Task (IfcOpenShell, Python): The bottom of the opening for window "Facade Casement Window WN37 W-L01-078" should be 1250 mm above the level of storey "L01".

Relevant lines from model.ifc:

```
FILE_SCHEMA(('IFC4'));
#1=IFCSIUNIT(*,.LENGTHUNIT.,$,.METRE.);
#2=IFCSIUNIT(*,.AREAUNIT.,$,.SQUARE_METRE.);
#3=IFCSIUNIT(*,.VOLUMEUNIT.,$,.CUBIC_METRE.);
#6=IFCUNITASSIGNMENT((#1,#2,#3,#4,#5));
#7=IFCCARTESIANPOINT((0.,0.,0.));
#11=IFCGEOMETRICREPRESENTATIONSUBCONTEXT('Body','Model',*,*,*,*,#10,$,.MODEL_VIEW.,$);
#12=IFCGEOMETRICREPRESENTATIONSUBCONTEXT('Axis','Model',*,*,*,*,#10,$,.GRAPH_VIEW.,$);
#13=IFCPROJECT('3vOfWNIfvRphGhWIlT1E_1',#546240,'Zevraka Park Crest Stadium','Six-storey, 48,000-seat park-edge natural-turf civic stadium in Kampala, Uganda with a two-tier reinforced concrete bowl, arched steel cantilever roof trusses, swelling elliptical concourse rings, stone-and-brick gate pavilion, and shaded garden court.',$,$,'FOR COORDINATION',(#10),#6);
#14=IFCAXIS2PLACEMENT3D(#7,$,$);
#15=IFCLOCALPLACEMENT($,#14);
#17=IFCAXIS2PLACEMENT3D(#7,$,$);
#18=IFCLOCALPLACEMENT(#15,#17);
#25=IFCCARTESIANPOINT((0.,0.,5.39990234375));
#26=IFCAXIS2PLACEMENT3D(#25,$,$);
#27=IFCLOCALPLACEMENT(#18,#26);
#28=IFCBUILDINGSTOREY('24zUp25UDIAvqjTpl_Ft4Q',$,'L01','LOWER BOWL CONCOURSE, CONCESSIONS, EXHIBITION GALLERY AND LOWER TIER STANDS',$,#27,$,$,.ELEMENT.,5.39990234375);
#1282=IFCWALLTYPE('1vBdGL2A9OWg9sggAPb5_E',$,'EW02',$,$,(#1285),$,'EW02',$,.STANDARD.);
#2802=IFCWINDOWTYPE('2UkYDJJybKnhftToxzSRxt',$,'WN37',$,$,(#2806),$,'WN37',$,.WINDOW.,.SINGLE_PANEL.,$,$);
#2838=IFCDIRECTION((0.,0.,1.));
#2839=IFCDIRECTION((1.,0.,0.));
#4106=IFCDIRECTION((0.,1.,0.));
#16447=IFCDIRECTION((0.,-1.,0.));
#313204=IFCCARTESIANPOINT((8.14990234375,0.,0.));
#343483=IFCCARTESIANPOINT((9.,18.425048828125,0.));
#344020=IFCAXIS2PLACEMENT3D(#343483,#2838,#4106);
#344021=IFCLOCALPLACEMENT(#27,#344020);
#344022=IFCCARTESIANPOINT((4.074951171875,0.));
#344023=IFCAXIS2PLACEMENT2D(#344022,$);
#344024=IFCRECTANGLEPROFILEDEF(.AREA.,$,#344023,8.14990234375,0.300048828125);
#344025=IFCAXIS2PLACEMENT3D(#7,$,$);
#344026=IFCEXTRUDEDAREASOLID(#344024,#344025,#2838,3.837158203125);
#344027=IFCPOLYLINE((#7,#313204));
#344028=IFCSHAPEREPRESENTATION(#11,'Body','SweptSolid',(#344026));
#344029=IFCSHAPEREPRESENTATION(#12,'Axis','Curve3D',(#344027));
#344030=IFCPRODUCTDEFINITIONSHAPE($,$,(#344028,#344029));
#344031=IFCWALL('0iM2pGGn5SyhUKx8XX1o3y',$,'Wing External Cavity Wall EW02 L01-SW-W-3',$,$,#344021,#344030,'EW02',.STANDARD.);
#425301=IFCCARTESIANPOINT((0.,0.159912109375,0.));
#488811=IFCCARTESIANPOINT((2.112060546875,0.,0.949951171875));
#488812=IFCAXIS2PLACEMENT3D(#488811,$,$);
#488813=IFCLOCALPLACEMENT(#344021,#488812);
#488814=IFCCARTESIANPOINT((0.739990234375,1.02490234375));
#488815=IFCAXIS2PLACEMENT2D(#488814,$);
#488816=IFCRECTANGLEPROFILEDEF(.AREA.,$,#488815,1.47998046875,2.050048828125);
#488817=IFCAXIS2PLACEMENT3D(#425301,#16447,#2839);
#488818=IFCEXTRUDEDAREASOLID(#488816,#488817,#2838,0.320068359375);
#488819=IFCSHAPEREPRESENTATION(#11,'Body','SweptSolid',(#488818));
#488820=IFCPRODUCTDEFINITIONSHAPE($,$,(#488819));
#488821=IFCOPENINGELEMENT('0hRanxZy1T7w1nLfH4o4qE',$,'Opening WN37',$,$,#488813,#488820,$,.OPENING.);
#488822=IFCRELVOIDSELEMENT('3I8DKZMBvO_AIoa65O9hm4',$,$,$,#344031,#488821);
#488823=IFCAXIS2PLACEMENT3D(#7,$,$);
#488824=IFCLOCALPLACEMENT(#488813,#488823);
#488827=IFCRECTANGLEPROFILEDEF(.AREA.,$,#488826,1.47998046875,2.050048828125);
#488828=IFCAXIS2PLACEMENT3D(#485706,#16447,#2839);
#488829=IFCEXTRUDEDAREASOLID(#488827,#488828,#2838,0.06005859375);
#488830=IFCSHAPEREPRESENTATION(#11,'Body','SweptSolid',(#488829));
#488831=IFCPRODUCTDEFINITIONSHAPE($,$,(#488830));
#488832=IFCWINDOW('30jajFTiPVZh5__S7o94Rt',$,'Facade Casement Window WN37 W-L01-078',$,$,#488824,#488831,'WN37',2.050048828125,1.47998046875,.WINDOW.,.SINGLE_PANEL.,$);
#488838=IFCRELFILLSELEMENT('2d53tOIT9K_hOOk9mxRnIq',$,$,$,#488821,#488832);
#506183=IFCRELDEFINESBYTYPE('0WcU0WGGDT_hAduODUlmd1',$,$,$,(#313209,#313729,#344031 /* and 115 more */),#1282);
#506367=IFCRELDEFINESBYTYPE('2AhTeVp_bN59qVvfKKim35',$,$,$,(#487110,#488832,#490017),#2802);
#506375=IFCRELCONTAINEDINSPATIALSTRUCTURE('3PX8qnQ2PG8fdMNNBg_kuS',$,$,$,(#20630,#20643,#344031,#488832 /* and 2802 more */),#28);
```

```python
import numpy as np
import ifcopenshell
import ifcopenshell.api.geometry
import ifcopenshell.geom
import ifcopenshell.util.element
import ifcopenshell.util.placement
import ifcopenshell.util.shape
import ifcopenshell.util.unit

model = ifcopenshell.open("model.ifc")
unit_scale = ifcopenshell.util.unit.calculate_unit_scale(model)

window = model.by_guid("30jajFTiPVZh5__S7o94Rt")
opening = window.FillsVoids[0].RelatingOpeningElement
storey = ifcopenshell.util.element.get_container(window, ifc_class="IfcBuildingStorey")
level = ifcopenshell.util.placement.get_local_placement(storey.ObjectPlacement)[2, 3]

# The opening's origin need not be at the sill, so measure its lowest point.
shape = ifcopenshell.geom.create_shape(ifcopenshell.geom.settings(), opening)
bottom = ifcopenshell.util.shape.get_shape_bottom_elevation(shape, shape.geometry) / unit_scale
dz = level + 1.25 - bottom

shift = np.array([0.0, 0.0, dz])
# The window is placed relative to its opening, so it follows when the opening moves.
matrix = ifcopenshell.util.placement.get_local_placement(opening.ObjectPlacement)
matrix[:3, 3] += shift
ifcopenshell.api.geometry.edit_object_placement(
    model, product=opening, matrix=matrix, is_si=False, should_transform_children=True
)

print(f"moved by {dz * unit_scale:+.3f} m")

model.write("model-out.ifc")
```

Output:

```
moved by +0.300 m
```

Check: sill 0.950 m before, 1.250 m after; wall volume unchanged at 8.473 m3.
